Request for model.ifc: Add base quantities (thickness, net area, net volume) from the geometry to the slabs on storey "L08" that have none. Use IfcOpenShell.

First a look at what the model holds.

```python
import ifcopenshell
import ifcopenshell.util.element
import ifcopenshell.util.unit

model = ifcopenshell.open("model.ifc")
print(model.schema)
for unit_type in ("LENGTHUNIT", "AREAUNIT", "VOLUMEUNIT"):
    print(unit_type, ifcopenshell.util.unit.calculate_unit_scale(model, unit_type))
storey = next(s for s in model.by_type("IfcBuildingStorey") if s.Name == "L08")
slabs = [e for e in ifcopenshell.util.element.get_decomposition(storey) if e.is_a("IfcSlab")]
for e in sorted(slabs, key=lambda e: e.id()):
    print(e.id(), e.is_a(), e.Name, list(ifcopenshell.util.element.get_psets(e, qtos_only=True)), sep=" | ")
```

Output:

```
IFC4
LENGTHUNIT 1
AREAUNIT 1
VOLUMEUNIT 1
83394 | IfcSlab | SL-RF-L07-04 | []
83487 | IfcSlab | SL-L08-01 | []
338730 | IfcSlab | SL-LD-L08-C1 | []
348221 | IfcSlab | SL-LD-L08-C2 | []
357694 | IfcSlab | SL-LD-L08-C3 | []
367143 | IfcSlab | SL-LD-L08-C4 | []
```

```python
import ifcopenshell
import ifcopenshell.api.pset
import ifcopenshell.geom
import ifcopenshell.util.element
import ifcopenshell.util.shape
import ifcopenshell.util.unit

model = ifcopenshell.open("model.ifc")
unit_scale = ifcopenshell.util.unit.calculate_unit_scale(model)
area_scale = ifcopenshell.util.unit.calculate_unit_scale(model, "AREAUNIT")
volume_scale = ifcopenshell.util.unit.calculate_unit_scale(model, "VOLUMEUNIT")
settings = ifcopenshell.geom.settings()

storey = next(s for s in model.by_type("IfcBuildingStorey") if s.Name == "L08")
slabs = [e for e in ifcopenshell.util.element.get_decomposition(storey) if e.is_a("IfcSlab")]

for e in sorted(slabs, key=lambda e: e.id()):
    if ifcopenshell.util.element.get_psets(e, qtos_only=True, should_inherit=False):
        continue
    # Geometry comes back in metres, in the element's own axes.
    shape = ifcopenshell.geom.create_shape(settings, e)
    values = {
        "Width": ifcopenshell.util.shape.get_z(shape.geometry) / unit_scale,
        "NetArea": ifcopenshell.util.shape.get_footprint_area(shape.geometry) / area_scale,
        "NetVolume": ifcopenshell.util.shape.get_volume(shape.geometry) / volume_scale,
    }
    qto = ifcopenshell.api.pset.add_qto(model, product=e, name="Qto_SlabBaseQuantities")
    ifcopenshell.api.pset.edit_qto(model, qto=qto, properties=values)
    print(e.id(), {k: round(v, 3) for k, v in values.items()})

model.write("model-out.ifc")
```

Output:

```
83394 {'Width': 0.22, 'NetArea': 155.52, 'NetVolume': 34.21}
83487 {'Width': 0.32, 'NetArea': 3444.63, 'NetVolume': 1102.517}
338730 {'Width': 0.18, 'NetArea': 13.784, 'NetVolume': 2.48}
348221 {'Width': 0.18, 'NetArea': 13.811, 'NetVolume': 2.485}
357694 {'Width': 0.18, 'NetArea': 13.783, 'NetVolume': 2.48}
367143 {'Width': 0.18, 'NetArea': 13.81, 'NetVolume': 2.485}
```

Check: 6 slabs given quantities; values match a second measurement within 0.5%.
